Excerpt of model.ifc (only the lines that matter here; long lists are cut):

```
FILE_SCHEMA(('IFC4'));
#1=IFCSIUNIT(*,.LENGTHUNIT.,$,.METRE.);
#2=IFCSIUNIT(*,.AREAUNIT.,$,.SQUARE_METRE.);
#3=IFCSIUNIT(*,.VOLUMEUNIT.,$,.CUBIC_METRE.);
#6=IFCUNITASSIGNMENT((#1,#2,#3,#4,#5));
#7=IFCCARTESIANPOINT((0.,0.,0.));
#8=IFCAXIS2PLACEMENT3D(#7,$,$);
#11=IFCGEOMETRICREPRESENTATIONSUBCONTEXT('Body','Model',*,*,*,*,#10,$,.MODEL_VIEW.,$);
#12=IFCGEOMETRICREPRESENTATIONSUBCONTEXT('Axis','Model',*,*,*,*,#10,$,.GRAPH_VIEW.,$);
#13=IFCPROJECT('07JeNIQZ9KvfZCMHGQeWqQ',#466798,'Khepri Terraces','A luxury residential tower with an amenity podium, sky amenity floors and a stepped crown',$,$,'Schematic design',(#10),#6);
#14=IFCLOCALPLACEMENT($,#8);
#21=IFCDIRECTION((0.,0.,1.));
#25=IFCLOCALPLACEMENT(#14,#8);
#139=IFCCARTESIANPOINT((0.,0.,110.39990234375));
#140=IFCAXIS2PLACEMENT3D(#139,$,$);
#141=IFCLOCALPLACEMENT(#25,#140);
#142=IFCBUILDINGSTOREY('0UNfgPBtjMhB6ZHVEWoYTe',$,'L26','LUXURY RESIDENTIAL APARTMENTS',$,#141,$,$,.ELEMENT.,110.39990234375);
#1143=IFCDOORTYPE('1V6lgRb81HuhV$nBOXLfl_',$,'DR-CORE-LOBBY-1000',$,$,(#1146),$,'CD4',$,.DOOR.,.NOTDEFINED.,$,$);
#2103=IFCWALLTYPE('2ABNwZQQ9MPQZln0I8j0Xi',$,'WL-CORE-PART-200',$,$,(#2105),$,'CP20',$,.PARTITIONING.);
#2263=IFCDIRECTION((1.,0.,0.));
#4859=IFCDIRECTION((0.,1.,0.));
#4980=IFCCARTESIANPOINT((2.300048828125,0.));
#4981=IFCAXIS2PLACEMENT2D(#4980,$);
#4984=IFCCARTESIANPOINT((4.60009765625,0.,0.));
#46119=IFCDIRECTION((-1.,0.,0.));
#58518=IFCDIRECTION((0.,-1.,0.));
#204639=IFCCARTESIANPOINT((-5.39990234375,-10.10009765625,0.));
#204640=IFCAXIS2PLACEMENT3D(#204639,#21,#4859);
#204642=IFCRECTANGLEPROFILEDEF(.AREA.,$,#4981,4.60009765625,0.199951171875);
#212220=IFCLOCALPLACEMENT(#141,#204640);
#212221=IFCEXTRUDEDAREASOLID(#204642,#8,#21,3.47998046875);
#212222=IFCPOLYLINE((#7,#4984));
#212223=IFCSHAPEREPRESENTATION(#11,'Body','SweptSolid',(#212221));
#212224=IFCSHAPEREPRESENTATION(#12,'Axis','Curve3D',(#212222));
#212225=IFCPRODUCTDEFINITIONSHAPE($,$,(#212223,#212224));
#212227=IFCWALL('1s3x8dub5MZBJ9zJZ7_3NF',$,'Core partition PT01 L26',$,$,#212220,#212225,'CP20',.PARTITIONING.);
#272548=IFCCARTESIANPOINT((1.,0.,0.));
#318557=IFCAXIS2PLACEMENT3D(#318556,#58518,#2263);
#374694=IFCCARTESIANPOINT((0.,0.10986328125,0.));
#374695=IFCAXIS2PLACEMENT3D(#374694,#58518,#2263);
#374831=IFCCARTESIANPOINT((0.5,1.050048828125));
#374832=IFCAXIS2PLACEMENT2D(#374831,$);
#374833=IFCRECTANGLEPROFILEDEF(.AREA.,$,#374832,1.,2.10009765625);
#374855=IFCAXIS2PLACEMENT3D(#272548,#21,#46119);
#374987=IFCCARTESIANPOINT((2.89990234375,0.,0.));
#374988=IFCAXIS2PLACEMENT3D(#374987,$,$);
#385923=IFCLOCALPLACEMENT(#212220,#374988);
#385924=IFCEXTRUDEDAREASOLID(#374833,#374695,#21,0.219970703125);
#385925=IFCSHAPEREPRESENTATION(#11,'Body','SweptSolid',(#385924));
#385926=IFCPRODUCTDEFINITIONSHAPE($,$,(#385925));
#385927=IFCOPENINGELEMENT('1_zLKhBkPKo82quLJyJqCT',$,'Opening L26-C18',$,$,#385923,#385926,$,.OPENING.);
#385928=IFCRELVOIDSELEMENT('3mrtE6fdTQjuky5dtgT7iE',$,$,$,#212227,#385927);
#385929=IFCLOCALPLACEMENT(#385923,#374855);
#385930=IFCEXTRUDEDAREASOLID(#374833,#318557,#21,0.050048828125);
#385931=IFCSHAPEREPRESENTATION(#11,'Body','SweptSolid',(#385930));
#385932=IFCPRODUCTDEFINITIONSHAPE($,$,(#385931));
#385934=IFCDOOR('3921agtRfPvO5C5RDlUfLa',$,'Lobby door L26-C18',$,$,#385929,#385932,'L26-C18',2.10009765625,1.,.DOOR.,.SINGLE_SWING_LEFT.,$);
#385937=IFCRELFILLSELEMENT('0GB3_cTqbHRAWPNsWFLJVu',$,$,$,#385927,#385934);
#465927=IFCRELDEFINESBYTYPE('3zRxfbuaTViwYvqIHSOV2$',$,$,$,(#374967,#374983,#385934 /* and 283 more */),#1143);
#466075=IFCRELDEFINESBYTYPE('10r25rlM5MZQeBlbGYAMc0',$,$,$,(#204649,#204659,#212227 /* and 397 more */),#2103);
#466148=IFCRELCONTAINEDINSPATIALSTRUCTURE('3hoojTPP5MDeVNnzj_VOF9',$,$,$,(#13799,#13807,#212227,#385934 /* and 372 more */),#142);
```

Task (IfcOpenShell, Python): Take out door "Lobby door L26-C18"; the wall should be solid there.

```python
import ifcopenshell
import ifcopenshell.api.feature
import ifcopenshell.api.root
import ifcopenshell.geom
import ifcopenshell.util.shape

model = ifcopenshell.open("model.ifc")
settings = ifcopenshell.geom.settings()


def volume(element):
    """Net volume in cubic metres, openings subtracted."""
    shape = ifcopenshell.geom.create_shape(settings, element)
    return ifcopenshell.util.shape.get_volume(shape.geometry)


door = model.by_guid("3921agtRfPvO5C5RDlUfLa")
opening = door.FillsVoids[0].RelatingOpeningElement
wall = opening.VoidsElements[0].RelatingBuildingElement
before = volume(wall)

ifcopenshell.api.root.remove_product(model, product=door)
ifcopenshell.api.feature.remove_feature(model, feature=opening)

after = volume(wall)

print(f"wall volume {before:.3f} -> {after:.3f} m3")

model.write("model-out.ifc")
```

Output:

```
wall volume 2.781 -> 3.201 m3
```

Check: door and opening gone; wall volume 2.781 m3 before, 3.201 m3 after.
